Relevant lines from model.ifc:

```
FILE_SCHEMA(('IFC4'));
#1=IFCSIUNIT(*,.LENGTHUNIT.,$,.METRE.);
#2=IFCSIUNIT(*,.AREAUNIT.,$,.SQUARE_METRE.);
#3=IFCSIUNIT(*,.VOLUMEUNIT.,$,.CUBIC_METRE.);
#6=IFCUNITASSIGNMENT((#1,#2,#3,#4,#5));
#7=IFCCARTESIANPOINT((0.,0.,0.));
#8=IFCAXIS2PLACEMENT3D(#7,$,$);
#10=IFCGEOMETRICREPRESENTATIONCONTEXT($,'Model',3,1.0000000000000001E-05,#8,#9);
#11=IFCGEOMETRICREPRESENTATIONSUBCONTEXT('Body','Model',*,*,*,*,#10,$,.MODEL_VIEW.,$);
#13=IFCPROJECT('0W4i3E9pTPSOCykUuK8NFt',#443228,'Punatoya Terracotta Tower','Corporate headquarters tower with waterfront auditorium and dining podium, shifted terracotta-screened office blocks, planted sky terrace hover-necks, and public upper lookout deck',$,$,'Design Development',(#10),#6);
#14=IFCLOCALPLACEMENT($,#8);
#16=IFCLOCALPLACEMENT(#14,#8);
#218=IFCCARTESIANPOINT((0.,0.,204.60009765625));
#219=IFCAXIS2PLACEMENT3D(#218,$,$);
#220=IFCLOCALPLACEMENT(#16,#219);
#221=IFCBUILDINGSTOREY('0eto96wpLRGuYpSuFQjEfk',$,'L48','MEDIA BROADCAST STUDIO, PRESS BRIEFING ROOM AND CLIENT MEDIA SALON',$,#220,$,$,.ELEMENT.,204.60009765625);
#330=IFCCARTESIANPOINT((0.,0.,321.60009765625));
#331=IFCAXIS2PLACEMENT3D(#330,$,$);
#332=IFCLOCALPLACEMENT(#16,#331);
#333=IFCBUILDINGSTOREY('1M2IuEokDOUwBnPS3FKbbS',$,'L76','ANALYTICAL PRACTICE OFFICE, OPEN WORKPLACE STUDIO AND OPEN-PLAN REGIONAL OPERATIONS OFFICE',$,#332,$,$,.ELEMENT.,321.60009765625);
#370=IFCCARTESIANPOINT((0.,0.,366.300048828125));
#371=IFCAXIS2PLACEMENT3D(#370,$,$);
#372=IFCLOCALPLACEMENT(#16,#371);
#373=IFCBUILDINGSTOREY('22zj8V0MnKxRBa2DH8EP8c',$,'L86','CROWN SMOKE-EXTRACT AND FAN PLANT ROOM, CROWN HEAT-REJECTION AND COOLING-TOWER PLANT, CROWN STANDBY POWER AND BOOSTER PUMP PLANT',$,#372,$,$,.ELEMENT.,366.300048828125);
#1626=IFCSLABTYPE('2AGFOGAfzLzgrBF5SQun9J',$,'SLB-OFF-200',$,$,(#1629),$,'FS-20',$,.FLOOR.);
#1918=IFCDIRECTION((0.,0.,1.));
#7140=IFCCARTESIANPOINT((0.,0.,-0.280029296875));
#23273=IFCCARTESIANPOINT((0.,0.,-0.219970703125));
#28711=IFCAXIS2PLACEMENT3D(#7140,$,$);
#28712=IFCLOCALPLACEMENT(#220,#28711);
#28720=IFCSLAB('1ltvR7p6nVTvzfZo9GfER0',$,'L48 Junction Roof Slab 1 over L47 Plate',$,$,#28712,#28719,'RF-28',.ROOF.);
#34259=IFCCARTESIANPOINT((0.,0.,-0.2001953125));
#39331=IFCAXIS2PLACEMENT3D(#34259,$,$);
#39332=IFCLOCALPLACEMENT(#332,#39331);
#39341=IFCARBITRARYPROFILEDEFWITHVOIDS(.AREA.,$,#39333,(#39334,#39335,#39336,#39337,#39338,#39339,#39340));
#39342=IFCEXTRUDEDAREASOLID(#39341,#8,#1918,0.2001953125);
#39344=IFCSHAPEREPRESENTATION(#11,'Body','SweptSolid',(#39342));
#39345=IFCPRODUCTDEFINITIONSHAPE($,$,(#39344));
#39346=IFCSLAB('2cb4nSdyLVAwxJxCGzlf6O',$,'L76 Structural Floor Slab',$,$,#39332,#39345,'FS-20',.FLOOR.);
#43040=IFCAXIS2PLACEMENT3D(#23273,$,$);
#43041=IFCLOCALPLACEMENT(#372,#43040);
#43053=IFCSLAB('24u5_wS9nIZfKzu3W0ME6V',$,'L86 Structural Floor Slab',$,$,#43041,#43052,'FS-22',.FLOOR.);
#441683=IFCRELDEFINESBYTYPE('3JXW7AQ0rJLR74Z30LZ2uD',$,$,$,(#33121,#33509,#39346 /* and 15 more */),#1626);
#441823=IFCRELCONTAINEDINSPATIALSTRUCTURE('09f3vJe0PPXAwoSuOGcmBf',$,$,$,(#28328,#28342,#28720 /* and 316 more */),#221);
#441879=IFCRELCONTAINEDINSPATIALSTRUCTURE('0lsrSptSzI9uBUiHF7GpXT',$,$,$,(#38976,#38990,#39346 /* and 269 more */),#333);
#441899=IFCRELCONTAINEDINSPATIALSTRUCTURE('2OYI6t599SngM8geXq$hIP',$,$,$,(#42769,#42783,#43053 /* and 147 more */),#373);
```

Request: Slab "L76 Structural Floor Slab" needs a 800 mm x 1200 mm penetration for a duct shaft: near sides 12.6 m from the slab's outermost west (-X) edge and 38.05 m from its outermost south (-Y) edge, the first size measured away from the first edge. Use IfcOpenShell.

```python
import numpy as np
import ifcopenshell
import ifcopenshell.api.feature
import ifcopenshell.api.geometry
import ifcopenshell.api.root
import ifcopenshell.geom
import ifcopenshell.util.placement
import ifcopenshell.util.representation
import ifcopenshell.util.shape
import ifcopenshell.util.unit

model = ifcopenshell.open("model.ifc")
unit_scale = ifcopenshell.util.unit.calculate_unit_scale(model)
settings = ifcopenshell.geom.settings()


def volume(element):
    """Net volume in cubic metres, openings subtracted."""
    shape = ifcopenshell.geom.create_shape(settings, element)
    return ifcopenshell.util.shape.get_volume(shape.geometry)


slab = model.by_id(39346)
before = volume(slab)

# Extent in the slab's own axes, in metres. The edges named are its -X and -Y sides.
slab_shape = ifcopenshell.geom.create_shape(settings, slab)
vertices = ifcopenshell.util.shape.get_vertices(slab_shape.geometry)
x_min, y_min, bottom = vertices.min(axis=0)
top = vertices[:, 2].max()

opening = ifcopenshell.api.root.create_entity(model, ifc_class="IfcOpeningElement", name="Duct shaft opening", predefined_type="OPENING")
context = ifcopenshell.util.representation.get_context(model, "Model", "Body", "MODEL_VIEW")
width, depth = 0.8, 1.2
outline = [(0.0, 0.0), (width, 0.0), (width, depth), (0.0, depth), (0.0, 0.0)]
# Overshoot both faces by 50 mm so the cut is clean.
shape = ifcopenshell.api.geometry.add_slab_representation(
    model, context=context, depth=top - bottom + 0.1, polyline=outline
)
ifcopenshell.api.geometry.assign_representation(model, product=opening, representation=shape)

matrix = ifcopenshell.util.placement.get_local_placement(slab.ObjectPlacement)
matrix[:, 3] = matrix @ np.append(np.array([x_min + 12.6, y_min + 38.05, bottom - 0.05]) / unit_scale, 1.0)
ifcopenshell.api.geometry.edit_object_placement(model, product=opening, matrix=matrix, is_si=False)
ifcopenshell.api.feature.add_feature(model, feature=opening, element=slab)

after = volume(slab)

print(f"slab volume {before:.3f} -> {after:.3f} m3")

model.write("model_v2.ifc")
```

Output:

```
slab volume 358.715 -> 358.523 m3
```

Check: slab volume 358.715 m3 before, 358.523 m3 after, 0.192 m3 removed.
